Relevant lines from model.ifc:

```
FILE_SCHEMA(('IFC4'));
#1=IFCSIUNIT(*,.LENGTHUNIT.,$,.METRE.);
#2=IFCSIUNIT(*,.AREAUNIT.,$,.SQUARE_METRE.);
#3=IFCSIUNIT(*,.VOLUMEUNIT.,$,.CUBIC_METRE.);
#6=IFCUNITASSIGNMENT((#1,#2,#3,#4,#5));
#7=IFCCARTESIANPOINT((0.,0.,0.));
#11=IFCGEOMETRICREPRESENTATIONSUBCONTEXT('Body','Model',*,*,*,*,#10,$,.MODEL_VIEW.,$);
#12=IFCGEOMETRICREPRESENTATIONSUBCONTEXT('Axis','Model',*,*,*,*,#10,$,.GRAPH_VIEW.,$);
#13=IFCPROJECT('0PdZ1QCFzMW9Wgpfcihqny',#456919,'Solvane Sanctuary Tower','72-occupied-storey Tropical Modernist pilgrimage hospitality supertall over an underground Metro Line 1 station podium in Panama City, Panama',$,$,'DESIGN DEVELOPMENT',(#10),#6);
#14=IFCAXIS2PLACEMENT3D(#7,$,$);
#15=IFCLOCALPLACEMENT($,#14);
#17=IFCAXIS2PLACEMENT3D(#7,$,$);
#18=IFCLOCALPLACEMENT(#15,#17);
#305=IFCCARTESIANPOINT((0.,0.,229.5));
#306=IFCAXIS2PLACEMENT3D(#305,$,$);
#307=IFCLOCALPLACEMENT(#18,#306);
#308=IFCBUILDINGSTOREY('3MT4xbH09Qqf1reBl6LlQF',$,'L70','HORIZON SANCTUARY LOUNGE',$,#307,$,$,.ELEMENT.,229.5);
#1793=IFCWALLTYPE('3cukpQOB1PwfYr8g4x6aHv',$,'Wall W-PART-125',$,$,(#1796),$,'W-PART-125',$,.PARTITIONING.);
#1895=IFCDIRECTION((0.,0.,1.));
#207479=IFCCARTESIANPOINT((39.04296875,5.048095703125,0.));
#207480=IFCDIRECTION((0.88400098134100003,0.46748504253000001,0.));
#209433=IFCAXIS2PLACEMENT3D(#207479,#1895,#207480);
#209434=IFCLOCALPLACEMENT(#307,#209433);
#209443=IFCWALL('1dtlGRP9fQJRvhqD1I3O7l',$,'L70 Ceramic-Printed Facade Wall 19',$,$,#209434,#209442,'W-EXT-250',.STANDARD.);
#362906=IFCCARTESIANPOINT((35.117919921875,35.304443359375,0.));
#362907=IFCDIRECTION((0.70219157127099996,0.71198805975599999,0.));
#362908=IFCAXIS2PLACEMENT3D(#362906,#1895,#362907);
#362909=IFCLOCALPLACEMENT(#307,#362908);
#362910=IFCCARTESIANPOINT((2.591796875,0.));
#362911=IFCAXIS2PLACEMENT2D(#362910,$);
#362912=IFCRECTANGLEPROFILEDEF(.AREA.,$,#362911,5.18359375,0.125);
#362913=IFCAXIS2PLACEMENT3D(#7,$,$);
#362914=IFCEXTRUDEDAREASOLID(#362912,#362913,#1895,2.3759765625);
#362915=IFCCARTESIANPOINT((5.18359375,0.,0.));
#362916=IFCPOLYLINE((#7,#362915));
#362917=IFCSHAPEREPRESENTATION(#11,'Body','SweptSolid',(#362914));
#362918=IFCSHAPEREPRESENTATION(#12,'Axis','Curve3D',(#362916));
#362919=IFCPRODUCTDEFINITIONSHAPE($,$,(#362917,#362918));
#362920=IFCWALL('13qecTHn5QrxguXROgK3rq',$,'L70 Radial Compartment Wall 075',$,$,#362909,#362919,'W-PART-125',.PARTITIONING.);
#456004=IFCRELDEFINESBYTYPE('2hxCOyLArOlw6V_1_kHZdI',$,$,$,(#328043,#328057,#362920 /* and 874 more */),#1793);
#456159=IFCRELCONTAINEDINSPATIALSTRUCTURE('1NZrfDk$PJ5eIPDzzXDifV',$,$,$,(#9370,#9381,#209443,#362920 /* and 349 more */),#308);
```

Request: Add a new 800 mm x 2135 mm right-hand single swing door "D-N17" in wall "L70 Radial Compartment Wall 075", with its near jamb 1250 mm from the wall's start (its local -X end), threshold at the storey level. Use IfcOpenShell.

```python
import numpy as np
import ifcopenshell
import ifcopenshell.api.feature
import ifcopenshell.api.geometry
import ifcopenshell.api.root
import ifcopenshell.api.spatial
import ifcopenshell.geom
import ifcopenshell.util.element
import ifcopenshell.util.placement
import ifcopenshell.util.representation
import ifcopenshell.util.shape
import ifcopenshell.util.unit

model = ifcopenshell.open("model.ifc")
unit_scale = ifcopenshell.util.unit.calculate_unit_scale(model)
settings = ifcopenshell.geom.settings()


def volume(element):
    """Net volume in cubic metres, openings subtracted."""
    shape = ifcopenshell.geom.create_shape(settings, element)
    return ifcopenshell.util.shape.get_volume(shape.geometry)


wall = model.by_id(362920)
storey = ifcopenshell.util.element.get_container(wall, ifc_class="IfcBuildingStorey")
context = ifcopenshell.util.representation.get_context(model, "Model", "Body", "MODEL_VIEW")
before = volume(wall)

width, height, from_end, sill = 0.8, 2.135, 1.25, 0.0  # metres

# The wall runs along its own X axis, and the end named is its -X end.
wall_shape = ifcopenshell.geom.create_shape(settings, wall)
x, y, z = ifcopenshell.util.shape.get_vertices(wall_shape.geometry).T
start = x.min() + from_end
face, thickness = float(y.min()), float(y.max() - y.min())
wall_matrix = ifcopenshell.util.placement.get_local_placement(wall.ObjectPlacement)
level = ifcopenshell.util.placement.get_local_placement(storey.ObjectPlacement)[2, 3]


def in_wall(x, y):
    """Placement at x, y metres in the wall's axes, at sill height."""
    matrix = wall_matrix.copy()
    matrix[:, 3] = wall_matrix @ np.array([x / unit_scale, y / unit_scale, 0.0, 1.0])
    matrix[2, 3] = level + sill / unit_scale
    return matrix


# Opening: a box that overshoots both wall faces by 50 mm.
opening = ifcopenshell.api.root.create_entity(model, ifc_class="IfcOpeningElement", predefined_type="OPENING")
box = ifcopenshell.api.geometry.add_wall_representation(
    model, context=context, length=width, height=height, thickness=thickness + 0.1
)
ifcopenshell.api.geometry.assign_representation(model, product=opening, representation=box)
ifcopenshell.api.geometry.edit_object_placement(model, product=opening, matrix=in_wall(start, face - 0.05), is_si=False)
ifcopenshell.api.feature.add_feature(model, feature=opening, element=wall)

door = ifcopenshell.api.root.create_entity(model, ifc_class="IfcDoor", name="D-N17", predefined_type="DOOR")
door.OverallWidth, door.OverallHeight = width / unit_scale, height / unit_scale
door.OperationType = "SINGLE_SWING_RIGHT"
body = ifcopenshell.api.geometry.add_door_representation(
    model,
    context=context,
    overall_width=door.OverallWidth,
    overall_height=door.OverallHeight,
    operation_type="SINGLE_SWING_RIGHT",
    lining_properties={"LiningDepth": thickness / unit_scale, "ThresholdDepth": thickness / unit_scale},
)
ifcopenshell.api.geometry.assign_representation(model, product=door, representation=body)
ifcopenshell.api.spatial.assign_container(model, products=[door], relating_structure=storey)
ifcopenshell.api.feature.add_filling(model, opening=opening, element=door)

# The lining spans the wall, so the door starts at the wall face.
ifcopenshell.api.geometry.edit_object_placement(model, product=door, matrix=in_wall(start, face), is_si=False)

after = volume(wall)

print(f"wall volume {before:.3f} -> {after:.3f} m3")

model.write("model_rev.ifc")
```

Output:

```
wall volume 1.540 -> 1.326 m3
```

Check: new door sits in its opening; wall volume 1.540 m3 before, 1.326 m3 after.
